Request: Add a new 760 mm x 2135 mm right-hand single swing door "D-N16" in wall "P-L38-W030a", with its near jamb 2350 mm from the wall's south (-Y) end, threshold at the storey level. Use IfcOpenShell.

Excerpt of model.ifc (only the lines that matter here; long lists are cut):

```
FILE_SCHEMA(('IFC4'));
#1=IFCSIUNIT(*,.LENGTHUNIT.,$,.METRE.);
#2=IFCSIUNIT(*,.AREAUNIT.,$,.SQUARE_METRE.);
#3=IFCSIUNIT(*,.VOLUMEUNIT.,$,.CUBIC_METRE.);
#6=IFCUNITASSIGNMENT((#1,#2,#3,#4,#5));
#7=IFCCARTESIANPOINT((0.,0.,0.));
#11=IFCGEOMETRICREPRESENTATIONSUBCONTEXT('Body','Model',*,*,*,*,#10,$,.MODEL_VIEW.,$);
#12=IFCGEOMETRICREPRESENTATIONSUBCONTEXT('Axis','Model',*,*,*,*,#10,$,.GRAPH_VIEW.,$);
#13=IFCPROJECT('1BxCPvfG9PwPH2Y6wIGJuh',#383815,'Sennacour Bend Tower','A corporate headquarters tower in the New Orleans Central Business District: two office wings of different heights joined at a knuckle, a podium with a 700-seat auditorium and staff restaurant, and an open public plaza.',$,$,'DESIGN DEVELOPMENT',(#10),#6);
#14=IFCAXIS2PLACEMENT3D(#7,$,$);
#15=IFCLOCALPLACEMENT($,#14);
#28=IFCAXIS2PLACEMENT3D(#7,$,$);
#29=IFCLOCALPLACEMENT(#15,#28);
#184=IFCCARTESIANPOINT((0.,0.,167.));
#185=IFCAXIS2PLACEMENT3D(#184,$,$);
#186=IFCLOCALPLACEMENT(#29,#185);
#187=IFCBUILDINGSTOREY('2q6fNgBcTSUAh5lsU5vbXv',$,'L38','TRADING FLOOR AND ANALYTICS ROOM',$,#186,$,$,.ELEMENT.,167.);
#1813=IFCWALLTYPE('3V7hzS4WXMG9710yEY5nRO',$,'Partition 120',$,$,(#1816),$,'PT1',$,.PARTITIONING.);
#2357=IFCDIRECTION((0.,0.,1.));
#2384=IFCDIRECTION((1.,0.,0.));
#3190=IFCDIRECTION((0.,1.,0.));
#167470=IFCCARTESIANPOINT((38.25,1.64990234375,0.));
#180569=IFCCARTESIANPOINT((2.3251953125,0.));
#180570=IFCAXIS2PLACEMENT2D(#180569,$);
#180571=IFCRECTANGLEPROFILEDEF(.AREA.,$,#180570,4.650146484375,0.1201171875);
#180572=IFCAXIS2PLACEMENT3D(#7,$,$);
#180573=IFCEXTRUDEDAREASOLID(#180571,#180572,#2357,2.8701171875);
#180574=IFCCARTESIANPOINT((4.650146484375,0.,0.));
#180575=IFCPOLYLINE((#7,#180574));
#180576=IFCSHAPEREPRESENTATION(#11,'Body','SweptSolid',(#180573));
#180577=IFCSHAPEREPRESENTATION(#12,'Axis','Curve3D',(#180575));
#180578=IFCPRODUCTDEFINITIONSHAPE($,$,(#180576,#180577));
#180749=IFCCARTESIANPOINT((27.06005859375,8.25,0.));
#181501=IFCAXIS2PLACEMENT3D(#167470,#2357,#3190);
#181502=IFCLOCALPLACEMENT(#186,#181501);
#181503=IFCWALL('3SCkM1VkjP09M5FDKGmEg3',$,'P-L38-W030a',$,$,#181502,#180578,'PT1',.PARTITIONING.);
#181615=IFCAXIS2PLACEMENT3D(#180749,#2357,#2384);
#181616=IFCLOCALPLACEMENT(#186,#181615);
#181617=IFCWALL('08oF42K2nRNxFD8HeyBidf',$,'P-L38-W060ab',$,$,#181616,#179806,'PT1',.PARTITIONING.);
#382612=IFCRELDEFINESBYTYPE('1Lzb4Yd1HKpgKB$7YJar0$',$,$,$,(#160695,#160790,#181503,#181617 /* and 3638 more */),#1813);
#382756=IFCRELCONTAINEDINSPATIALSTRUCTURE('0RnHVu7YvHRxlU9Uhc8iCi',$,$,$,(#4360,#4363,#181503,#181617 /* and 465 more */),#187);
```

```python
import numpy as np
import ifcopenshell
import ifcopenshell.api.feature
import ifcopenshell.api.geometry
import ifcopenshell.api.root
import ifcopenshell.api.spatial
import ifcopenshell.geom
import ifcopenshell.util.element
import ifcopenshell.util.placement
import ifcopenshell.util.representation
import ifcopenshell.util.shape
import ifcopenshell.util.unit

model = ifcopenshell.open("model.ifc")
unit_scale = ifcopenshell.util.unit.calculate_unit_scale(model)
settings = ifcopenshell.geom.settings()


def volume(element):
    """Net volume in cubic metres, openings subtracted."""
    shape = ifcopenshell.geom.create_shape(settings, element)
    return ifcopenshell.util.shape.get_volume(shape.geometry)


wall = model.by_guid("3SCkM1VkjP09M5FDKGmEg3")
storey = ifcopenshell.util.element.get_container(wall, ifc_class="IfcBuildingStorey")
context = ifcopenshell.util.representation.get_context(model, "Model", "Body", "MODEL_VIEW")
before = volume(wall)

width, height, from_end, sill = 0.76, 2.135, 2.35, 0.0  # metres

# The wall runs along its own X axis, and the end named is its -X end.
wall_shape = ifcopenshell.geom.create_shape(settings, wall)
x, y, z = ifcopenshell.util.shape.get_vertices(wall_shape.geometry).T
start = x.min() + from_end
face, thickness = float(y.min()), float(y.max() - y.min())
wall_matrix = ifcopenshell.util.placement.get_local_placement(wall.ObjectPlacement)
level = ifcopenshell.util.placement.get_local_placement(storey.ObjectPlacement)[2, 3]


def in_wall(x, y):
    """Placement at x, y metres in the wall's axes, at sill height."""
    matrix = wall_matrix.copy()
    matrix[:, 3] = wall_matrix @ np.array([x / unit_scale, y / unit_scale, 0.0, 1.0])
    matrix[2, 3] = level + sill / unit_scale
    return matrix


# Opening: a box that overshoots both wall faces by 50 mm.
opening = ifcopenshell.api.root.create_entity(model, ifc_class="IfcOpeningElement", predefined_type="OPENING")
box = ifcopenshell.api.geometry.add_wall_representation(
    model, context=context, length=width, height=height, thickness=thickness + 0.1
)
ifcopenshell.api.geometry.assign_representation(model, product=opening, representation=box)
ifcopenshell.api.geometry.edit_object_placement(model, product=opening, matrix=in_wall(start, face - 0.05), is_si=False)
ifcopenshell.api.feature.add_feature(model, feature=opening, element=wall)

door = ifcopenshell.api.root.create_entity(model, ifc_class="IfcDoor", name="D-N16", predefined_type="DOOR")
door.OverallWidth, door.OverallHeight = width / unit_scale, height / unit_scale
door.OperationType = "SINGLE_SWING_RIGHT"
body = ifcopenshell.api.geometry.add_door_representation(
    model,
    context=context,
    overall_width=door.OverallWidth,
    overall_height=door.OverallHeight,
    operation_type="SINGLE_SWING_RIGHT",
    lining_properties={"LiningDepth": thickness / unit_scale, "ThresholdDepth": thickness / unit_scale},
)
ifcopenshell.api.geometry.assign_representation(model, product=door, representation=body)
ifcopenshell.api.spatial.assign_container(model, products=[door], relating_structure=storey)
ifcopenshell.api.feature.add_filling(model, opening=opening, element=door)

# The lining spans the wall, so the door starts at the wall face.
ifcopenshell.api.geometry.edit_object_placement(model, product=door, matrix=in_wall(start, face), is_si=False)

after = volume(wall)

print(f"wall volume {before:.3f} -> {after:.3f} m3")

model.write("model_edited.ifc")
```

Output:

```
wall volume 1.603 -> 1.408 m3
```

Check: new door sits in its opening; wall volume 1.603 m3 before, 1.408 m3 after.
